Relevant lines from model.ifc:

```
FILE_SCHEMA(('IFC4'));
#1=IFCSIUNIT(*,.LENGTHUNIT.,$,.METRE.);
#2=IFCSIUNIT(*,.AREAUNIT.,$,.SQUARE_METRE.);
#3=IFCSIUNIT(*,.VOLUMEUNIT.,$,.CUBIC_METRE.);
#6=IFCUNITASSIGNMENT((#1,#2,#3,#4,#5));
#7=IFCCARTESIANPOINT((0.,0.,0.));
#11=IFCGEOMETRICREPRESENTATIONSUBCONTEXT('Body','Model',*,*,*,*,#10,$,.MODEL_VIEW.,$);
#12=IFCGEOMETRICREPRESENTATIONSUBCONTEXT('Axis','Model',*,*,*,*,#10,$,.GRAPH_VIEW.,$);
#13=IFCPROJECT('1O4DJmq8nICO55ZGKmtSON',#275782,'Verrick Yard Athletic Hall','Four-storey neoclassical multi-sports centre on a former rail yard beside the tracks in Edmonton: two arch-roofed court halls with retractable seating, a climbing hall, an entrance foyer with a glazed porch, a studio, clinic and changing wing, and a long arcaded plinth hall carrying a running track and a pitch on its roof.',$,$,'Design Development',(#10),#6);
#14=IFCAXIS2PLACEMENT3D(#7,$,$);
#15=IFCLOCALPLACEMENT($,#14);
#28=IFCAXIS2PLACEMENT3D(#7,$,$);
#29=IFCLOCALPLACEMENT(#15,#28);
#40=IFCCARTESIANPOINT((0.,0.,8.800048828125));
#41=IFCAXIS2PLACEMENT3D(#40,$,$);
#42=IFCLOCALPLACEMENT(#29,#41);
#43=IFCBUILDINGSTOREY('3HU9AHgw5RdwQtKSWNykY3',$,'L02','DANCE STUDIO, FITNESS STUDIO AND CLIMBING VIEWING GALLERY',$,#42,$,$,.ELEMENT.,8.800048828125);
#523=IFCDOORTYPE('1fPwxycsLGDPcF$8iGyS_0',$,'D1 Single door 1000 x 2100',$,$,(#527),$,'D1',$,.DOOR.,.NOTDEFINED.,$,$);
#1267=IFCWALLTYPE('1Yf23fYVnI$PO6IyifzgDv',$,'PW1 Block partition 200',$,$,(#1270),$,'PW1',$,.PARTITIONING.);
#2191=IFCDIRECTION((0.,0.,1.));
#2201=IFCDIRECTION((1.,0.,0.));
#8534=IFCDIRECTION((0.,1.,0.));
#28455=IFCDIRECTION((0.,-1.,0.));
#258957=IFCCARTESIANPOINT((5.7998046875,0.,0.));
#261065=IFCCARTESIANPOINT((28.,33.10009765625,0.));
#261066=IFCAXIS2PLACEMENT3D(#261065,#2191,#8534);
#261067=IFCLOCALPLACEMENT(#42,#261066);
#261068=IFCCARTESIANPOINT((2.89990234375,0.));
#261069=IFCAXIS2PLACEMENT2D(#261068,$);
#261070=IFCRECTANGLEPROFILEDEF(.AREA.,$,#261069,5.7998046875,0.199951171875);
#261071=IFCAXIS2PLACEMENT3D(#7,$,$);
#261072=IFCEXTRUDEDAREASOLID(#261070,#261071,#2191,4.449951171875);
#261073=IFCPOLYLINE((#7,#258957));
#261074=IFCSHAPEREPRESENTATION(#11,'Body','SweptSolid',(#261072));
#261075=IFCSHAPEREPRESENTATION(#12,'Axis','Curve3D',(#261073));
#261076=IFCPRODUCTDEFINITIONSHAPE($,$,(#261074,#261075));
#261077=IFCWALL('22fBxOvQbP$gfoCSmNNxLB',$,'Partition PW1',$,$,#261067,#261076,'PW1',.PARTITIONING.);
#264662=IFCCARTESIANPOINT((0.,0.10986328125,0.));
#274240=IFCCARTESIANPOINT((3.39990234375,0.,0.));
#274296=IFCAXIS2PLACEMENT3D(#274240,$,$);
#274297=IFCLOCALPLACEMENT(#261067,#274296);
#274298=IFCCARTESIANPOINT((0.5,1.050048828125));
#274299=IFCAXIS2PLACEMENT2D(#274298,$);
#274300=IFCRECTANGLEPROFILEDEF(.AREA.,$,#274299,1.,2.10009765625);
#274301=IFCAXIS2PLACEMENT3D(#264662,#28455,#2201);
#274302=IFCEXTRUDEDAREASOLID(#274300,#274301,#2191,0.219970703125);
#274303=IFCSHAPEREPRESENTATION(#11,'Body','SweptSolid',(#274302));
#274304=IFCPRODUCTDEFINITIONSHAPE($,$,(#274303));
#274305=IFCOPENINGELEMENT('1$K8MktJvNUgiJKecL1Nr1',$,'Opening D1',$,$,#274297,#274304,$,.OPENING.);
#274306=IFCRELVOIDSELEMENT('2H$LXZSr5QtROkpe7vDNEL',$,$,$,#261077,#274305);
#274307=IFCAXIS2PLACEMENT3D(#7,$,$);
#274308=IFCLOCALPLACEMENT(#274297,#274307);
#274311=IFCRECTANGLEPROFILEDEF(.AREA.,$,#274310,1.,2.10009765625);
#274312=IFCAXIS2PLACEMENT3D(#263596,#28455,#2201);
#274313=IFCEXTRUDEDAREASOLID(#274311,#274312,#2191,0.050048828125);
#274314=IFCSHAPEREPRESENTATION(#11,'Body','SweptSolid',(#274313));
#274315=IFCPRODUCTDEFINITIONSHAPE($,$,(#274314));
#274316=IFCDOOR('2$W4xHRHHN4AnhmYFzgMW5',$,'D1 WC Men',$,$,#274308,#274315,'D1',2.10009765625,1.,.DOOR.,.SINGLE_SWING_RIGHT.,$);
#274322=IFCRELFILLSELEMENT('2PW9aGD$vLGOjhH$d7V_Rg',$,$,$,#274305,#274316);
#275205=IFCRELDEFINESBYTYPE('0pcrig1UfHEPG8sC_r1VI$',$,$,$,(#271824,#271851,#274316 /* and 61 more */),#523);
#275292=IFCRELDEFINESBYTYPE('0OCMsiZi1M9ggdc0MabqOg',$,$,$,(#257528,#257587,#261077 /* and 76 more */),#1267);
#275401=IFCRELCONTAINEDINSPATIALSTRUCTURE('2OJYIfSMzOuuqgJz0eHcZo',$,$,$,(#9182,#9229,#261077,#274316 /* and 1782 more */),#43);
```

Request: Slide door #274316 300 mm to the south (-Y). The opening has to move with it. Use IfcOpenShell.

```python
import ifcopenshell
import ifcopenshell.api.geometry
import ifcopenshell.util.placement
import ifcopenshell.util.unit

model = ifcopenshell.open("model.ifc")
unit_scale = ifcopenshell.util.unit.calculate_unit_scale(model)

door = model.by_id(274316)
opening = door.FillsVoids[0].RelatingOpeningElement
wall = opening.VoidsElements[0].RelatingBuildingElement

wall_matrix = ifcopenshell.util.placement.get_local_placement(wall.ObjectPlacement)
shift = wall_matrix[:3, 0] * -0.3 / unit_scale
before = ifcopenshell.util.placement.get_local_placement(door.ObjectPlacement)[:3, 3].copy()

# The door is placed relative to its opening, so it follows when the opening moves.
matrix = ifcopenshell.util.placement.get_local_placement(opening.ObjectPlacement)
matrix[:3, 3] += shift
ifcopenshell.api.geometry.edit_object_placement(
    model, product=opening, matrix=matrix, is_si=False, should_transform_children=True
)

after = ifcopenshell.util.placement.get_local_placement(door.ObjectPlacement)[:3, 3]
print("door moved by", (after - before).round(3) + 0.0)

model.write("model_updated.ifc")
```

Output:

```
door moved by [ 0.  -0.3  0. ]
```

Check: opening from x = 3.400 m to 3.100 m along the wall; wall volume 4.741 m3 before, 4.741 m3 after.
